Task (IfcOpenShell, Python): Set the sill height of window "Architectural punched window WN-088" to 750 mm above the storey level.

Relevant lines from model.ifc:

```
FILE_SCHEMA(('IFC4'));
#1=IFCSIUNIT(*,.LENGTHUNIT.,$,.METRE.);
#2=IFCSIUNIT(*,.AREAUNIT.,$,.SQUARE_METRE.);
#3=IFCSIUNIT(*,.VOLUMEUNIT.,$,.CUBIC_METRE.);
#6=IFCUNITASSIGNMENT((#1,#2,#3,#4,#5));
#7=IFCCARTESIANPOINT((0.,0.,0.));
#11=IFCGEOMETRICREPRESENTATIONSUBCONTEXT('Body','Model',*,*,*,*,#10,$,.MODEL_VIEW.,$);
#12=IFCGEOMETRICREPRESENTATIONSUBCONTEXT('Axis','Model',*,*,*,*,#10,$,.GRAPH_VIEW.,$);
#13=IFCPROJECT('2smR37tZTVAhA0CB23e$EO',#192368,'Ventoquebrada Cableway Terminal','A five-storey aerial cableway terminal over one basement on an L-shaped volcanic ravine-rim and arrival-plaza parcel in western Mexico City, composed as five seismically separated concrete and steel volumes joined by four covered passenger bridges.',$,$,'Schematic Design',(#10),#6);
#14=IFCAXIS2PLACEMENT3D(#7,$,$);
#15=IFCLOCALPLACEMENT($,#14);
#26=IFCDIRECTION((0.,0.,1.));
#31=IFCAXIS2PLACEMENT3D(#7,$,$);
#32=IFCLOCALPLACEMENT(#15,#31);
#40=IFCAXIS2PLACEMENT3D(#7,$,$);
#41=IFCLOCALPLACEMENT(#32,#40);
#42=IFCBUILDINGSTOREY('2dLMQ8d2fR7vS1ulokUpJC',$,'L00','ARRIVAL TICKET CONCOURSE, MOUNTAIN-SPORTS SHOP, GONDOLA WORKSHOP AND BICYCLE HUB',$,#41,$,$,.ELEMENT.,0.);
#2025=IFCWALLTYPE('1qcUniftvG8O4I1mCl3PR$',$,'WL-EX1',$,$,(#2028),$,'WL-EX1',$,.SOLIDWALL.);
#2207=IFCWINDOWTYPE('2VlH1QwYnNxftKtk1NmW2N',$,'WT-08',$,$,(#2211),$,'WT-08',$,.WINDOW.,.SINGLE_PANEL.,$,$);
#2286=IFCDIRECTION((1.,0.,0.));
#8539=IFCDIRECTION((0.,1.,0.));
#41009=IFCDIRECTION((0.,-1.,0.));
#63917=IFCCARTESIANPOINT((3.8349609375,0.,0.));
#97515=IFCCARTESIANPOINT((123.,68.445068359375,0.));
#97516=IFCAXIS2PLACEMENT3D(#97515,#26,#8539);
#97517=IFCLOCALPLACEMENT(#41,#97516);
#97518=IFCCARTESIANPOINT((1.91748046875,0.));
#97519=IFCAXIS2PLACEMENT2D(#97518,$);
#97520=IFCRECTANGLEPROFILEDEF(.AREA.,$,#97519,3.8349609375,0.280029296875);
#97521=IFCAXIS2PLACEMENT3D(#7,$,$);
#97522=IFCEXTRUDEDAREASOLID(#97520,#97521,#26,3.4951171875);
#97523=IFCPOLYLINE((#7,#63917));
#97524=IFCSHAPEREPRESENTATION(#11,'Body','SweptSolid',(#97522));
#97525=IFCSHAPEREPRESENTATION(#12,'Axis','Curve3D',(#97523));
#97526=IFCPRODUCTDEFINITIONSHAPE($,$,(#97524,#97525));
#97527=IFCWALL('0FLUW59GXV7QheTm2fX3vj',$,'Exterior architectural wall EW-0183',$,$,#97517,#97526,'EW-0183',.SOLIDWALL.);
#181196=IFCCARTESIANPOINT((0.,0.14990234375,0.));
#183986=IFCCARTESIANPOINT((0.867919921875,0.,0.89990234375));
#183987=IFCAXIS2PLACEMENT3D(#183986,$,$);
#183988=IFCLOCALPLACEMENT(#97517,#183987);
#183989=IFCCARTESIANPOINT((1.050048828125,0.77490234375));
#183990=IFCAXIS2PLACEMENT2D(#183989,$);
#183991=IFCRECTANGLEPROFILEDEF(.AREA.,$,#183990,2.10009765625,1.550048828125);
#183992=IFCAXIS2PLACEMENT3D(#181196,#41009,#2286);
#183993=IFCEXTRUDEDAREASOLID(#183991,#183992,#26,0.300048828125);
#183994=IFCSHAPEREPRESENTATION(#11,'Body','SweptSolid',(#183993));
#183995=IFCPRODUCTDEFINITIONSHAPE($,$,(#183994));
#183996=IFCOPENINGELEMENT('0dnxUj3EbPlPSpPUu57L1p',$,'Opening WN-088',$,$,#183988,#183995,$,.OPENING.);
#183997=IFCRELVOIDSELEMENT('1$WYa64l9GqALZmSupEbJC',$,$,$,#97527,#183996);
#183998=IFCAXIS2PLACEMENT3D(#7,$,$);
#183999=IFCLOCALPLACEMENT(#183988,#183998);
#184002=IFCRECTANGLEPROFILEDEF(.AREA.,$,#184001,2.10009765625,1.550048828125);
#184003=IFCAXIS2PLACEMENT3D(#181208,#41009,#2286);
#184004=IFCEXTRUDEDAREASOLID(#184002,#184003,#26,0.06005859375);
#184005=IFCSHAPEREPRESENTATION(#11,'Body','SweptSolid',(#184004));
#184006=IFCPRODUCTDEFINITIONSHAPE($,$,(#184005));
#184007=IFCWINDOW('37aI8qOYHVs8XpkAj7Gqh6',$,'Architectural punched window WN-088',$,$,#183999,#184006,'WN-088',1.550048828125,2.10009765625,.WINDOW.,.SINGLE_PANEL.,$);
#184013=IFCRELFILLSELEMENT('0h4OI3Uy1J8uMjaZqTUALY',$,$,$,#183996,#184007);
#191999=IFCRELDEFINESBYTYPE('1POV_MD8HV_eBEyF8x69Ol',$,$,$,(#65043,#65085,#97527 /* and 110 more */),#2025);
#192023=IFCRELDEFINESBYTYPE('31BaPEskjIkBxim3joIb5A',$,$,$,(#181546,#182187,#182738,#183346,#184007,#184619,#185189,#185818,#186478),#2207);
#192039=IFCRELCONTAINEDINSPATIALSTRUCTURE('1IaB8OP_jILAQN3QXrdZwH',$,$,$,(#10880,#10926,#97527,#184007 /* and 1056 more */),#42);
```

```python
import numpy as np
import ifcopenshell
import ifcopenshell.api.geometry
import ifcopenshell.geom
import ifcopenshell.util.element
import ifcopenshell.util.placement
import ifcopenshell.util.shape
import ifcopenshell.util.unit

model = ifcopenshell.open("model.ifc")
unit_scale = ifcopenshell.util.unit.calculate_unit_scale(model)

window = model.by_guid("37aI8qOYHVs8XpkAj7Gqh6")
opening = window.FillsVoids[0].RelatingOpeningElement
storey = ifcopenshell.util.element.get_container(window, ifc_class="IfcBuildingStorey")
level = ifcopenshell.util.placement.get_local_placement(storey.ObjectPlacement)[2, 3]

# The opening's origin need not be at the sill, so measure its lowest point.
shape = ifcopenshell.geom.create_shape(ifcopenshell.geom.settings(), opening)
bottom = ifcopenshell.util.shape.get_shape_bottom_elevation(shape, shape.geometry) / unit_scale
dz = level + 0.75 - bottom

shift = np.array([0.0, 0.0, dz])
# The window is placed relative to its opening, so it follows when the opening moves.
matrix = ifcopenshell.util.placement.get_local_placement(opening.ObjectPlacement)
matrix[:3, 3] += shift
ifcopenshell.api.geometry.edit_object_placement(
    model, product=opening, matrix=matrix, is_si=False, should_transform_children=True
)

print(f"moved by {dz * unit_scale:+.3f} m")

model.write("model_rev.ifc")
```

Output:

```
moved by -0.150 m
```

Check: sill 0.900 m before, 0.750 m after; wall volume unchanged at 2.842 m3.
